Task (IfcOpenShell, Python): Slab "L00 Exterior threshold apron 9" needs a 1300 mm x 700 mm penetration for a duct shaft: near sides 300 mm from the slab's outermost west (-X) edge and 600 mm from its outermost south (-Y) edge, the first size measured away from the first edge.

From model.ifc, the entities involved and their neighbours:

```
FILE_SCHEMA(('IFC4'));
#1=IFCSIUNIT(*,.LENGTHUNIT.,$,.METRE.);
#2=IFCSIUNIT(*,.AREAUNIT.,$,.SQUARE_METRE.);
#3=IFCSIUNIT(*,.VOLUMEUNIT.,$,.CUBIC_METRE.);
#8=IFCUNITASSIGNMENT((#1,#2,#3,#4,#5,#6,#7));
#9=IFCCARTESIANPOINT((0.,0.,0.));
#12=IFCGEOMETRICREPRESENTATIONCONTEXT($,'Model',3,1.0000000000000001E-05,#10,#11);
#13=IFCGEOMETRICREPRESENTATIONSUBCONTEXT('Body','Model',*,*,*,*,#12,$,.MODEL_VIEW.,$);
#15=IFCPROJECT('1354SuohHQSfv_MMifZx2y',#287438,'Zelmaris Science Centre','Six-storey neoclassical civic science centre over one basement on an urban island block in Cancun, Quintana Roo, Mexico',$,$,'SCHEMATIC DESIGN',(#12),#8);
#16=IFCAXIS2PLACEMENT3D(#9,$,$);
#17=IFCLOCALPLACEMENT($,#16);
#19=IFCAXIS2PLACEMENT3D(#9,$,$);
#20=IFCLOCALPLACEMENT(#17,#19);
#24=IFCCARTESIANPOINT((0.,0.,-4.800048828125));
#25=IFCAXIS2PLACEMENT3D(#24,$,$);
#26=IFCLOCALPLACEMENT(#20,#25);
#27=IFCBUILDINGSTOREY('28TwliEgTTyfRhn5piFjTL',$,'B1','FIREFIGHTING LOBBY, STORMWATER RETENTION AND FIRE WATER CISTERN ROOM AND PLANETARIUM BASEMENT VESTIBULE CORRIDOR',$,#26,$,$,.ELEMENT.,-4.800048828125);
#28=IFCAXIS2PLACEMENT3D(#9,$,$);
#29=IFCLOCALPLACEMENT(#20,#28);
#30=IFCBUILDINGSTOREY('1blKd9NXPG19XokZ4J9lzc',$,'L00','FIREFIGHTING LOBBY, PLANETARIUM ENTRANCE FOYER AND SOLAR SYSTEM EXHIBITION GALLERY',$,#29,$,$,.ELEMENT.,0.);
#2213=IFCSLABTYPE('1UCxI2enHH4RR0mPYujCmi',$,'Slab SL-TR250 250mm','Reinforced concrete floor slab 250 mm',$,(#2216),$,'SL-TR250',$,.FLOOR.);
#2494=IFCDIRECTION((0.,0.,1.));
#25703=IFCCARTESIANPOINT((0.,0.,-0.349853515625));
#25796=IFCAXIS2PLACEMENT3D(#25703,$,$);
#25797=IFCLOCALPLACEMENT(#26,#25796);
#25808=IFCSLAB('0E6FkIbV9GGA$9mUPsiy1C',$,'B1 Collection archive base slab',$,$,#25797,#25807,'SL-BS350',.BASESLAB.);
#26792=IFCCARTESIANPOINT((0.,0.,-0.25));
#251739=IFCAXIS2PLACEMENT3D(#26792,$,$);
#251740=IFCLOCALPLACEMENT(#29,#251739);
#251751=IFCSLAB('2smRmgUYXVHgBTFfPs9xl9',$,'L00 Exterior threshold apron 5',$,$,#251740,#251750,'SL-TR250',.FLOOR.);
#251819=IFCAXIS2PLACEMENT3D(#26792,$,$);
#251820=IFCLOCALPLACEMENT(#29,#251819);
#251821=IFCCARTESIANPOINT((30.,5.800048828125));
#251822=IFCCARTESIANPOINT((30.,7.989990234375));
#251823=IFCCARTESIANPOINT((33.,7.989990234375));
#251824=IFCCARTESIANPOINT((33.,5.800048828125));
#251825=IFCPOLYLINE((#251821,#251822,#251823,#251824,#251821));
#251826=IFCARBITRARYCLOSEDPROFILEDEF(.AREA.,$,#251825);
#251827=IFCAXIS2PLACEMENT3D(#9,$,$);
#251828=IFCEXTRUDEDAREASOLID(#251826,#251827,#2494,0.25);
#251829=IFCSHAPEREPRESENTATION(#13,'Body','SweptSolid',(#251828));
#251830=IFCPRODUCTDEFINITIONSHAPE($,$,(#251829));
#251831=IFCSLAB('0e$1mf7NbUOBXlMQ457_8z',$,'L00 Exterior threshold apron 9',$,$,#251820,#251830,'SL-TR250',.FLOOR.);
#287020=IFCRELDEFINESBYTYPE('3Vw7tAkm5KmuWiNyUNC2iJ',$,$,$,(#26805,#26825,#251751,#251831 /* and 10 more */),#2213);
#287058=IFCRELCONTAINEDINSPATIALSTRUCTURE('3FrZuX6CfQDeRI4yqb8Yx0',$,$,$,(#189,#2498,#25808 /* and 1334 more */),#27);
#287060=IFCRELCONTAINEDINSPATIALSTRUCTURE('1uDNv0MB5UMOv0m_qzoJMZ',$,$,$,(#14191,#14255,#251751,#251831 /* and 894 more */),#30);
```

```python
import numpy as np
import ifcopenshell
import ifcopenshell.api.feature
import ifcopenshell.api.geometry
import ifcopenshell.api.root
import ifcopenshell.geom
import ifcopenshell.util.placement
import ifcopenshell.util.representation
import ifcopenshell.util.shape
import ifcopenshell.util.unit

model = ifcopenshell.open("model.ifc")
unit_scale = ifcopenshell.util.unit.calculate_unit_scale(model)
settings = ifcopenshell.geom.settings()


def volume(element):
    """Net volume in cubic metres, openings subtracted."""
    shape = ifcopenshell.geom.create_shape(settings, element)
    return ifcopenshell.util.shape.get_volume(shape.geometry)


slab = model.by_guid("0e$1mf7NbUOBXlMQ457_8z")
before = volume(slab)

# Extent in the slab's own axes, in metres. The edges named are its -X and -Y sides.
slab_shape = ifcopenshell.geom.create_shape(settings, slab)
vertices = ifcopenshell.util.shape.get_vertices(slab_shape.geometry)
x_min, y_min, bottom = vertices.min(axis=0)
top = vertices[:, 2].max()

opening = ifcopenshell.api.root.create_entity(model, ifc_class="IfcOpeningElement", name="Duct shaft opening", predefined_type="OPENING")
context = ifcopenshell.util.representation.get_context(model, "Model", "Body", "MODEL_VIEW")
width, depth = 1.3, 0.7
outline = [(0.0, 0.0), (width, 0.0), (width, depth), (0.0, depth), (0.0, 0.0)]
# Overshoot both faces by 50 mm so the cut is clean.
shape = ifcopenshell.api.geometry.add_slab_representation(
    model, context=context, depth=top - bottom + 0.1, polyline=outline
)
ifcopenshell.api.geometry.assign_representation(model, product=opening, representation=shape)

matrix = ifcopenshell.util.placement.get_local_placement(slab.ObjectPlacement)
matrix[:, 3] = matrix @ np.append(np.array([x_min + 0.3, y_min + 0.6, bottom - 0.05]) / unit_scale, 1.0)
ifcopenshell.api.geometry.edit_object_placement(model, product=opening, matrix=matrix, is_si=False)
ifcopenshell.api.feature.add_feature(model, feature=opening, element=slab)

after = volume(slab)

print(f"slab volume {before:.3f} -> {after:.3f} m3")

model.write("model-out.ifc")
```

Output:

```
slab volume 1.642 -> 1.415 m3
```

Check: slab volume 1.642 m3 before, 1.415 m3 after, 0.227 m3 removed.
